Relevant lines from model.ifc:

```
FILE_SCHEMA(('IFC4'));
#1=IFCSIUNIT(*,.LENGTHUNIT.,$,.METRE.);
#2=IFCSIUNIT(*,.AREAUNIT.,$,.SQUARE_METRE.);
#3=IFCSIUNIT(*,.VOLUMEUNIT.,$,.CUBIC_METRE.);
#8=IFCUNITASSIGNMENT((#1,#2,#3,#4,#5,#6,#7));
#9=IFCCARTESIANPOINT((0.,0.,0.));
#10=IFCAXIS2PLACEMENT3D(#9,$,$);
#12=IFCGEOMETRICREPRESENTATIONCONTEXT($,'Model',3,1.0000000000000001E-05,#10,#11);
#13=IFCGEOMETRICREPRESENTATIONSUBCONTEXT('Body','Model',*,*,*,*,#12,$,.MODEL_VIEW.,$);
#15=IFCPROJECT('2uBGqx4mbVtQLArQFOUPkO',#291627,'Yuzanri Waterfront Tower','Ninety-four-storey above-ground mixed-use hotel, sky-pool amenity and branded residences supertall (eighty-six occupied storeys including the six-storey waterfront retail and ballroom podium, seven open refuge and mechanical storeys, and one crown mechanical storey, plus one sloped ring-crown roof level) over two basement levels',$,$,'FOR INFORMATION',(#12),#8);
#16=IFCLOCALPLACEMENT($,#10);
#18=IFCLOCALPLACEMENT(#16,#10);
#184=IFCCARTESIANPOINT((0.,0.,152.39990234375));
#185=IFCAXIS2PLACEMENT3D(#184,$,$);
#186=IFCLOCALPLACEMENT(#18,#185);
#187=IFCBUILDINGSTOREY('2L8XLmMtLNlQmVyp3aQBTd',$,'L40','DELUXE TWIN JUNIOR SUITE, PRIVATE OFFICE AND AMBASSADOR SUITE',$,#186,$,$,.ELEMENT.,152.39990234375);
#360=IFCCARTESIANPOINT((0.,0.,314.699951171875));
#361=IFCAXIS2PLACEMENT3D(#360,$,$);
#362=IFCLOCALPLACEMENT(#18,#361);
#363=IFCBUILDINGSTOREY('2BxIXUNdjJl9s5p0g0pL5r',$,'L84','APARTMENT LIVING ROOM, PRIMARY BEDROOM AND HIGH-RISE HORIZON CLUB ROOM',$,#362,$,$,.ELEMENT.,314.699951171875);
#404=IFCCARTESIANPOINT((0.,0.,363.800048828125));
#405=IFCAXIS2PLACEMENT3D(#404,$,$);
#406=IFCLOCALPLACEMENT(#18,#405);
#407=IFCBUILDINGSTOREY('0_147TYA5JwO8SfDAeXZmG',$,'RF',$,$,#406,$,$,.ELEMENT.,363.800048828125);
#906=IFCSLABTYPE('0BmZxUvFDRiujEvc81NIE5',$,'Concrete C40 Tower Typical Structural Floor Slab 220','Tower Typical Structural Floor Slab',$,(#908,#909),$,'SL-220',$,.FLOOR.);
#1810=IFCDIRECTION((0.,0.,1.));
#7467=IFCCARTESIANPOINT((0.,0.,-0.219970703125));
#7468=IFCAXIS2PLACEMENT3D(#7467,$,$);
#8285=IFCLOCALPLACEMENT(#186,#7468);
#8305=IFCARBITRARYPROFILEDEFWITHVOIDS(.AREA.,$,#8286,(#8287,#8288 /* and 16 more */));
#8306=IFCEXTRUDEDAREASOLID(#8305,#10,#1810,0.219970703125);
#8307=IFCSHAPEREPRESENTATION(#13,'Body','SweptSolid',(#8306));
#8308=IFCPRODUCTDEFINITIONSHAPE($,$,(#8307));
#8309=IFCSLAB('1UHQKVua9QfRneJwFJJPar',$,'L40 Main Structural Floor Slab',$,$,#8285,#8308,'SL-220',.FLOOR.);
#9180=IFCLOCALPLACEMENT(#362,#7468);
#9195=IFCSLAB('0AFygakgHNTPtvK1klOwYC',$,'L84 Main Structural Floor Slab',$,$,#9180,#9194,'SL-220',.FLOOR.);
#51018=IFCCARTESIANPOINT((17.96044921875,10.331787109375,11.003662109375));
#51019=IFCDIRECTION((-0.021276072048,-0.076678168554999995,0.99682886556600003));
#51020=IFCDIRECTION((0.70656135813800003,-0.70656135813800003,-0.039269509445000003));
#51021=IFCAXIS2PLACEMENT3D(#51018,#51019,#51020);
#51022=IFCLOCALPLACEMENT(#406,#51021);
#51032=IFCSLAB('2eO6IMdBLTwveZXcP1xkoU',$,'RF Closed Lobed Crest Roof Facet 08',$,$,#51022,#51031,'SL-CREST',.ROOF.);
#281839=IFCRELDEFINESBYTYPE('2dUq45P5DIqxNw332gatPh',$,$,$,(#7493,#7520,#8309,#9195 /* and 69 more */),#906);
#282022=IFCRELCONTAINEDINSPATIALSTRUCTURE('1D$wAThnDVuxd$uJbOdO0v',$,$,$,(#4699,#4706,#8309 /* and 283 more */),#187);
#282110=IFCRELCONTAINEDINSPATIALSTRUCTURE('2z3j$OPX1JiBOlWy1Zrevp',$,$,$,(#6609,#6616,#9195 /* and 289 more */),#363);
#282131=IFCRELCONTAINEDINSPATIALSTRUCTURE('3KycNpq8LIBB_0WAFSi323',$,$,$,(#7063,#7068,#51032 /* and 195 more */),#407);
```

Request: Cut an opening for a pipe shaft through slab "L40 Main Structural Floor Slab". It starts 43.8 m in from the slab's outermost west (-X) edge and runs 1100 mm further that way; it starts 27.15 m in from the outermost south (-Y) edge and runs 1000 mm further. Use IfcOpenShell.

```python
import numpy as np
import ifcopenshell
import ifcopenshell.api.feature
import ifcopenshell.api.geometry
import ifcopenshell.api.root
import ifcopenshell.geom
import ifcopenshell.util.placement
import ifcopenshell.util.representation
import ifcopenshell.util.shape
import ifcopenshell.util.unit

model = ifcopenshell.open("model.ifc")
unit_scale = ifcopenshell.util.unit.calculate_unit_scale(model)
settings = ifcopenshell.geom.settings()


def volume(element):
    """Net volume in cubic metres, openings subtracted."""
    shape = ifcopenshell.geom.create_shape(settings, element)
    return ifcopenshell.util.shape.get_volume(shape.geometry)


slab = model.by_id(8309)
before = volume(slab)

# Extent in the slab's own axes, in metres. The edges named are its -X and -Y sides.
slab_shape = ifcopenshell.geom.create_shape(settings, slab)
vertices = ifcopenshell.util.shape.get_vertices(slab_shape.geometry)
x_min, y_min, bottom = vertices.min(axis=0)
top = vertices[:, 2].max()

opening = ifcopenshell.api.root.create_entity(model, ifc_class="IfcOpeningElement", name="Pipe shaft opening", predefined_type="OPENING")
context = ifcopenshell.util.representation.get_context(model, "Model", "Body", "MODEL_VIEW")
width, depth = 1.1, 1
outline = [(0.0, 0.0), (width, 0.0), (width, depth), (0.0, depth), (0.0, 0.0)]
# Overshoot both faces by 50 mm so the cut is clean.
shape = ifcopenshell.api.geometry.add_slab_representation(
    model, context=context, depth=top - bottom + 0.1, polyline=outline
)
ifcopenshell.api.geometry.assign_representation(model, product=opening, representation=shape)

matrix = ifcopenshell.util.placement.get_local_placement(slab.ObjectPlacement)
matrix[:, 3] = matrix @ np.append(np.array([x_min + 43.8, y_min + 27.15, bottom - 0.05]) / unit_scale, 1.0)
ifcopenshell.api.geometry.edit_object_placement(model, product=opening, matrix=matrix, is_si=False)
ifcopenshell.api.feature.add_feature(model, feature=opening, element=slab)

after = volume(slab)

print(f"slab volume {before:.3f} -> {after:.3f} m3")

model.write("model_rev.ifc")
```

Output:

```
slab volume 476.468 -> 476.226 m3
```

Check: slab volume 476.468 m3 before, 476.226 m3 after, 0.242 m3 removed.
